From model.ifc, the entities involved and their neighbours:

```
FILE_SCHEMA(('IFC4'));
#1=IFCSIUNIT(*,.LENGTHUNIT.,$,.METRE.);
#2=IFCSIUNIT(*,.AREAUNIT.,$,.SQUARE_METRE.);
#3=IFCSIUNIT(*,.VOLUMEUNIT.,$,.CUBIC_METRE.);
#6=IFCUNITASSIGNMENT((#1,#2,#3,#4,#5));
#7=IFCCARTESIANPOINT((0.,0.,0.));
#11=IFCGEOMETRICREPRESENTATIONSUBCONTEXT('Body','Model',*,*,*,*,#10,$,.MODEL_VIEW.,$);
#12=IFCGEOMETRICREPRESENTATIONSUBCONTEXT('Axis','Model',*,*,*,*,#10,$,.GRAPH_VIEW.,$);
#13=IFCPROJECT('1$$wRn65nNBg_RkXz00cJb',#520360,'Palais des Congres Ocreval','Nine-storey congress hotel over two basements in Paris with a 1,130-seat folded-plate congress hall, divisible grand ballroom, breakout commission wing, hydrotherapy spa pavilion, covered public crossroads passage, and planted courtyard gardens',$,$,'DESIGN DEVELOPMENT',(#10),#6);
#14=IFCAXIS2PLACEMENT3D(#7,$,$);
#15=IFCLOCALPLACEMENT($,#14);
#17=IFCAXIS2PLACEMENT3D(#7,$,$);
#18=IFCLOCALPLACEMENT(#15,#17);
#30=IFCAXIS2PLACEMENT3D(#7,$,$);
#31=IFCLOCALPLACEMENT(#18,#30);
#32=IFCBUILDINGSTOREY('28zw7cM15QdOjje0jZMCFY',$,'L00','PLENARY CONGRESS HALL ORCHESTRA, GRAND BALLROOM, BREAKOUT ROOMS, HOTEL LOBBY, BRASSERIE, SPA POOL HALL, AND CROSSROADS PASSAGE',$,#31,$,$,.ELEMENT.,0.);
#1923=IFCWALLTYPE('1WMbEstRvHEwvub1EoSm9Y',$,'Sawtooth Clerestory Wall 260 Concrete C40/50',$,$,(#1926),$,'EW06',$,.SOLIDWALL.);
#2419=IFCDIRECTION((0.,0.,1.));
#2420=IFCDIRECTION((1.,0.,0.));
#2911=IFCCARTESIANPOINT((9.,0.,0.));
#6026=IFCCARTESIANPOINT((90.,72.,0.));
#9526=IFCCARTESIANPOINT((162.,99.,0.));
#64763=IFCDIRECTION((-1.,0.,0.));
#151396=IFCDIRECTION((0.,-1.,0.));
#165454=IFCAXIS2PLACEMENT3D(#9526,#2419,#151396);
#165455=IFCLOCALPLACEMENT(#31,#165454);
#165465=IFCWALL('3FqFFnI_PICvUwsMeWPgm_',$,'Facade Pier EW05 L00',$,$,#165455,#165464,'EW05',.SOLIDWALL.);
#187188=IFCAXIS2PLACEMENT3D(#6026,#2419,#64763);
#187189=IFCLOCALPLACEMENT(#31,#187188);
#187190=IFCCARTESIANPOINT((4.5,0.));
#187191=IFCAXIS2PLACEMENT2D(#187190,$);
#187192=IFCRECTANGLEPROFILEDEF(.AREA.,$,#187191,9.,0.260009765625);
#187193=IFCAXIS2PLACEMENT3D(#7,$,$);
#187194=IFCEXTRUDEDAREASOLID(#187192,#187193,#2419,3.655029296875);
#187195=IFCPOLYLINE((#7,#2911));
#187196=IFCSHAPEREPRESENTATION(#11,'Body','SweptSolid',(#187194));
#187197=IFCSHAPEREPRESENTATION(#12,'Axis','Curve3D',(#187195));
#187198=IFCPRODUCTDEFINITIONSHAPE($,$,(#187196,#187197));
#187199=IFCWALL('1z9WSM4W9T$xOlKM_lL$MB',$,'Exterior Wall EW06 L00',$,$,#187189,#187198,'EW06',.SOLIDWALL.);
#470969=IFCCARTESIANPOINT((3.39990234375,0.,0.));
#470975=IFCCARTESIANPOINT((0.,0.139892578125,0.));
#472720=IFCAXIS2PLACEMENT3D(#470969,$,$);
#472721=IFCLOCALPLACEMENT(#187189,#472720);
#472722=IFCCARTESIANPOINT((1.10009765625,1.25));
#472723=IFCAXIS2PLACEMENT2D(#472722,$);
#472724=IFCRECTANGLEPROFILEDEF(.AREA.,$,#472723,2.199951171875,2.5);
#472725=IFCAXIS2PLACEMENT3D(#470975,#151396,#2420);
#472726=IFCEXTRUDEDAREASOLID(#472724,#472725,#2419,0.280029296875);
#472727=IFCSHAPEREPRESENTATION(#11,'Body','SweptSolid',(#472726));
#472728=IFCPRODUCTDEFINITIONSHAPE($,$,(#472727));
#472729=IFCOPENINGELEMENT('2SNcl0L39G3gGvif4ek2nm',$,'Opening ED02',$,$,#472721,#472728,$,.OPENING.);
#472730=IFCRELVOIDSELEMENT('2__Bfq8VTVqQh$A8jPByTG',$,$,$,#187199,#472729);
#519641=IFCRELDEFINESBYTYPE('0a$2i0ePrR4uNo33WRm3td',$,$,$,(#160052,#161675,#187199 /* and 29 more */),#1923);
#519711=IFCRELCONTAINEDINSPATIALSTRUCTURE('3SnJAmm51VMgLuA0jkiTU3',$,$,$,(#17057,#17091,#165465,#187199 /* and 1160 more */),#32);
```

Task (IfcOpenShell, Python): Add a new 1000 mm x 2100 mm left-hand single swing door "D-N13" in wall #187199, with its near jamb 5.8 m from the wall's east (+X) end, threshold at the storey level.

```python
import numpy as np
import ifcopenshell
import ifcopenshell.api.feature
import ifcopenshell.api.geometry
import ifcopenshell.api.root
import ifcopenshell.api.spatial
import ifcopenshell.geom
import ifcopenshell.util.element
import ifcopenshell.util.placement
import ifcopenshell.util.representation
import ifcopenshell.util.shape
import ifcopenshell.util.unit

model = ifcopenshell.open("model.ifc")
unit_scale = ifcopenshell.util.unit.calculate_unit_scale(model)
settings = ifcopenshell.geom.settings()


def volume(element):
    """Net volume in cubic metres, openings subtracted."""
    shape = ifcopenshell.geom.create_shape(settings, element)
    return ifcopenshell.util.shape.get_volume(shape.geometry)


wall = model.by_guid("1z9WSM4W9T$xOlKM_lL$MB")
storey = ifcopenshell.util.element.get_container(wall, ifc_class="IfcBuildingStorey")
context = ifcopenshell.util.representation.get_context(model, "Model", "Body", "MODEL_VIEW")
before = volume(wall)

width, height, from_end, sill = 1, 2.1, 5.8, 0.0  # metres

# The wall runs along its own X axis, and the end named is its -X end.
wall_shape = ifcopenshell.geom.create_shape(settings, wall)
x, y, z = ifcopenshell.util.shape.get_vertices(wall_shape.geometry).T
start = x.min() + from_end
face, thickness = float(y.min()), float(y.max() - y.min())
wall_matrix = ifcopenshell.util.placement.get_local_placement(wall.ObjectPlacement)
level = ifcopenshell.util.placement.get_local_placement(storey.ObjectPlacement)[2, 3]


def in_wall(x, y):
    """Placement at x, y metres in the wall's axes, at sill height."""
    matrix = wall_matrix.copy()
    matrix[:, 3] = wall_matrix @ np.array([x / unit_scale, y / unit_scale, 0.0, 1.0])
    matrix[2, 3] = level + sill / unit_scale
    return matrix


# Opening: a box that overshoots both wall faces by 50 mm.
opening = ifcopenshell.api.root.create_entity(model, ifc_class="IfcOpeningElement", predefined_type="OPENING")
box = ifcopenshell.api.geometry.add_wall_representation(
    model, context=context, length=width, height=height, thickness=thickness + 0.1
)
ifcopenshell.api.geometry.assign_representation(model, product=opening, representation=box)
ifcopenshell.api.geometry.edit_object_placement(model, product=opening, matrix=in_wall(start, face - 0.05), is_si=False)
ifcopenshell.api.feature.add_feature(model, feature=opening, element=wall)

door = ifcopenshell.api.root.create_entity(model, ifc_class="IfcDoor", name="D-N13", predefined_type="DOOR")
door.OverallWidth, door.OverallHeight = width / unit_scale, height / unit_scale
door.OperationType = "SINGLE_SWING_LEFT"
body = ifcopenshell.api.geometry.add_door_representation(
    model,
    context=context,
    overall_width=door.OverallWidth,
    overall_height=door.OverallHeight,
    operation_type="SINGLE_SWING_LEFT",
    lining_properties={"LiningDepth": thickness / unit_scale, "ThresholdDepth": thickness / unit_scale},
)
ifcopenshell.api.geometry.assign_representation(model, product=door, representation=body)
ifcopenshell.api.spatial.assign_container(model, products=[door], relating_structure=storey)
ifcopenshell.api.feature.add_filling(model, opening=opening, element=door)

# The lining spans the wall, so the door starts at the wall face.
ifcopenshell.api.geometry.edit_object_placement(model, product=door, matrix=in_wall(start, face), is_si=False)

after = volume(wall)

print(f"wall volume {before:.3f} -> {after:.3f} m3")

model.write("model_updated.ifc")
```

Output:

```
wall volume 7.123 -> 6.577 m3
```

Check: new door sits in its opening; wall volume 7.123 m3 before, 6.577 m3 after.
